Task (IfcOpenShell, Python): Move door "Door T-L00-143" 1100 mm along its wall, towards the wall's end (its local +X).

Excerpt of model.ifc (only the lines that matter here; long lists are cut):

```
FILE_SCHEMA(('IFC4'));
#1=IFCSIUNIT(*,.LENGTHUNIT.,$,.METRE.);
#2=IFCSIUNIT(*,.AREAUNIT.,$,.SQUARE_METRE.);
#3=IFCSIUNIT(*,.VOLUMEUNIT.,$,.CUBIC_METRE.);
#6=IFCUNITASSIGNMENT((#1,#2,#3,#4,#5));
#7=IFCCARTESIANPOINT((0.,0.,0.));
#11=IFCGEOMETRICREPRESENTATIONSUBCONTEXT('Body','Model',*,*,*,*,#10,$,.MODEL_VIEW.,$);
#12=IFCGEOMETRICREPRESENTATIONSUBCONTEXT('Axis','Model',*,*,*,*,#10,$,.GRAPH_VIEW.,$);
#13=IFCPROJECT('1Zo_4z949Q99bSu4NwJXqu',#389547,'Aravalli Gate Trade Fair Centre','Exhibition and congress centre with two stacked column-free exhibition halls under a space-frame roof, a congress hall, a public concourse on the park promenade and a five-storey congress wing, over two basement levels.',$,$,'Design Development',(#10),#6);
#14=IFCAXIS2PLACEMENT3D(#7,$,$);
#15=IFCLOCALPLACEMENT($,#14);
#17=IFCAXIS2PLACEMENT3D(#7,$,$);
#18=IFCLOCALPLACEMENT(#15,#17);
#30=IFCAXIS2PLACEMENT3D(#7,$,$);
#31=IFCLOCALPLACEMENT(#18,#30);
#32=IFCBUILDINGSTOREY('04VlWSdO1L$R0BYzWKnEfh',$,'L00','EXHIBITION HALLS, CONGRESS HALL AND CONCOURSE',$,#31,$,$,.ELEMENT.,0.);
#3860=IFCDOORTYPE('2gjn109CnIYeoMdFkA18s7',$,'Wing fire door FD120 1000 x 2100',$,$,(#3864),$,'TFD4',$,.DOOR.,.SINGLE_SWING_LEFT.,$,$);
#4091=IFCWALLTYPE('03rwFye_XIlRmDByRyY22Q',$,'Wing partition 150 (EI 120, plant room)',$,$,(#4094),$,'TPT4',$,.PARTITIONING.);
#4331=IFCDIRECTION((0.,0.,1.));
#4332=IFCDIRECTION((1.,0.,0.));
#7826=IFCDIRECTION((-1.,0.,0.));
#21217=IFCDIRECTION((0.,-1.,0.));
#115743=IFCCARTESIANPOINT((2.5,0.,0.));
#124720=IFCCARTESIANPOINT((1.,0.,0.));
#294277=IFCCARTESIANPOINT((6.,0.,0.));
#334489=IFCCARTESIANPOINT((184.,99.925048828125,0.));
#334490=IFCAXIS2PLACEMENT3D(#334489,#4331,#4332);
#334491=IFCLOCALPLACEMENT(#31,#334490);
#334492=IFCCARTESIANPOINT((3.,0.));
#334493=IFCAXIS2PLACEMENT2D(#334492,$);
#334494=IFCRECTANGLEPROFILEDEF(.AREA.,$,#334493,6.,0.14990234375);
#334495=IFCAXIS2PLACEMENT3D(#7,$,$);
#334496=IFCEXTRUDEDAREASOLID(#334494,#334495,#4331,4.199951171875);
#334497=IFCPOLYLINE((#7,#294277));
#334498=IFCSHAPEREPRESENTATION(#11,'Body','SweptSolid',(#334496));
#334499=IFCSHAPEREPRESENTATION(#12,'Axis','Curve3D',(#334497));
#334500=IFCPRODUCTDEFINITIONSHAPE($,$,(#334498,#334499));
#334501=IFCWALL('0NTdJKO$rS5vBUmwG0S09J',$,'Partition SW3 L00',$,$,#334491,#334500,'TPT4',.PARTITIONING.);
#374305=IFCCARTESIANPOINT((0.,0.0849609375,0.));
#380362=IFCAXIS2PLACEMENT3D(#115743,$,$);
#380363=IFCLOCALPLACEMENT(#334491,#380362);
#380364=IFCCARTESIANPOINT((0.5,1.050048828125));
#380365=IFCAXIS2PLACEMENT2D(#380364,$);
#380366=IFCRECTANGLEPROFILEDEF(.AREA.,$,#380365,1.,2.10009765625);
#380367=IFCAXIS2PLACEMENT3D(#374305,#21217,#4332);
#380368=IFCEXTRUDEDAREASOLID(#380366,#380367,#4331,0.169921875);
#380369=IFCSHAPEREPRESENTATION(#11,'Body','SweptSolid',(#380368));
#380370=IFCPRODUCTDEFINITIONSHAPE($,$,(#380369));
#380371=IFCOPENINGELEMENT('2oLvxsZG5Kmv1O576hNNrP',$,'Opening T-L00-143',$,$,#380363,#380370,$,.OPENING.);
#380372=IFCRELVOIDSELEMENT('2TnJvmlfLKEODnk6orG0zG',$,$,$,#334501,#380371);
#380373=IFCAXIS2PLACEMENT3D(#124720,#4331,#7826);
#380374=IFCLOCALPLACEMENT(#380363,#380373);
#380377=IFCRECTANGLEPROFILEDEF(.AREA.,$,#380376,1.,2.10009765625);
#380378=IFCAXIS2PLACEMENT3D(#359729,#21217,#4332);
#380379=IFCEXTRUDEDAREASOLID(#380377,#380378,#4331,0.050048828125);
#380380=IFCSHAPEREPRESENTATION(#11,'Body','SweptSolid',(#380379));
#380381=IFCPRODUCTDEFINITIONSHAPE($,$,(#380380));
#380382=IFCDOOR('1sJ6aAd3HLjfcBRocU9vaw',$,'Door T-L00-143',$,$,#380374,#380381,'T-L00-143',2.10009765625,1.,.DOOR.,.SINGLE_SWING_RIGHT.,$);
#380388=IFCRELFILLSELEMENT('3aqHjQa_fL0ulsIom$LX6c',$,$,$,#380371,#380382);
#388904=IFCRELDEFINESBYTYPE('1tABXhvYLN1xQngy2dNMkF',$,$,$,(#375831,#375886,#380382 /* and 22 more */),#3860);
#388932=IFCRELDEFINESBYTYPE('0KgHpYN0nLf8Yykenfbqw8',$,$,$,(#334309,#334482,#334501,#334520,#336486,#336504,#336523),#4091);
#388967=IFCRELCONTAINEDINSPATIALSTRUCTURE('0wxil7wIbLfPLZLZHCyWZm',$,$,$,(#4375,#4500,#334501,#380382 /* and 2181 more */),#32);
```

```python
import ifcopenshell
import ifcopenshell.api.geometry
import ifcopenshell.util.placement
import ifcopenshell.util.unit

model = ifcopenshell.open("model.ifc")
unit_scale = ifcopenshell.util.unit.calculate_unit_scale(model)

door = model.by_guid("1sJ6aAd3HLjfcBRocU9vaw")
opening = door.FillsVoids[0].RelatingOpeningElement
wall = opening.VoidsElements[0].RelatingBuildingElement

wall_matrix = ifcopenshell.util.placement.get_local_placement(wall.ObjectPlacement)
shift = wall_matrix[:3, 0] * 1.1 / unit_scale
before = ifcopenshell.util.placement.get_local_placement(door.ObjectPlacement)[:3, 3].copy()

# The door is placed relative to its opening, so it follows when the opening moves.
matrix = ifcopenshell.util.placement.get_local_placement(opening.ObjectPlacement)
matrix[:3, 3] += shift
ifcopenshell.api.geometry.edit_object_placement(
    model, product=opening, matrix=matrix, is_si=False, should_transform_children=True
)

after = ifcopenshell.util.placement.get_local_placement(door.ObjectPlacement)[:3, 3]
print("door moved by", (after - before).round(3) + 0.0)

model.write("model_updated.ifc")
```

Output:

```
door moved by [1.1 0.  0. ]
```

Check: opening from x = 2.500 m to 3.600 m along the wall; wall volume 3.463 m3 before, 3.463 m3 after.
